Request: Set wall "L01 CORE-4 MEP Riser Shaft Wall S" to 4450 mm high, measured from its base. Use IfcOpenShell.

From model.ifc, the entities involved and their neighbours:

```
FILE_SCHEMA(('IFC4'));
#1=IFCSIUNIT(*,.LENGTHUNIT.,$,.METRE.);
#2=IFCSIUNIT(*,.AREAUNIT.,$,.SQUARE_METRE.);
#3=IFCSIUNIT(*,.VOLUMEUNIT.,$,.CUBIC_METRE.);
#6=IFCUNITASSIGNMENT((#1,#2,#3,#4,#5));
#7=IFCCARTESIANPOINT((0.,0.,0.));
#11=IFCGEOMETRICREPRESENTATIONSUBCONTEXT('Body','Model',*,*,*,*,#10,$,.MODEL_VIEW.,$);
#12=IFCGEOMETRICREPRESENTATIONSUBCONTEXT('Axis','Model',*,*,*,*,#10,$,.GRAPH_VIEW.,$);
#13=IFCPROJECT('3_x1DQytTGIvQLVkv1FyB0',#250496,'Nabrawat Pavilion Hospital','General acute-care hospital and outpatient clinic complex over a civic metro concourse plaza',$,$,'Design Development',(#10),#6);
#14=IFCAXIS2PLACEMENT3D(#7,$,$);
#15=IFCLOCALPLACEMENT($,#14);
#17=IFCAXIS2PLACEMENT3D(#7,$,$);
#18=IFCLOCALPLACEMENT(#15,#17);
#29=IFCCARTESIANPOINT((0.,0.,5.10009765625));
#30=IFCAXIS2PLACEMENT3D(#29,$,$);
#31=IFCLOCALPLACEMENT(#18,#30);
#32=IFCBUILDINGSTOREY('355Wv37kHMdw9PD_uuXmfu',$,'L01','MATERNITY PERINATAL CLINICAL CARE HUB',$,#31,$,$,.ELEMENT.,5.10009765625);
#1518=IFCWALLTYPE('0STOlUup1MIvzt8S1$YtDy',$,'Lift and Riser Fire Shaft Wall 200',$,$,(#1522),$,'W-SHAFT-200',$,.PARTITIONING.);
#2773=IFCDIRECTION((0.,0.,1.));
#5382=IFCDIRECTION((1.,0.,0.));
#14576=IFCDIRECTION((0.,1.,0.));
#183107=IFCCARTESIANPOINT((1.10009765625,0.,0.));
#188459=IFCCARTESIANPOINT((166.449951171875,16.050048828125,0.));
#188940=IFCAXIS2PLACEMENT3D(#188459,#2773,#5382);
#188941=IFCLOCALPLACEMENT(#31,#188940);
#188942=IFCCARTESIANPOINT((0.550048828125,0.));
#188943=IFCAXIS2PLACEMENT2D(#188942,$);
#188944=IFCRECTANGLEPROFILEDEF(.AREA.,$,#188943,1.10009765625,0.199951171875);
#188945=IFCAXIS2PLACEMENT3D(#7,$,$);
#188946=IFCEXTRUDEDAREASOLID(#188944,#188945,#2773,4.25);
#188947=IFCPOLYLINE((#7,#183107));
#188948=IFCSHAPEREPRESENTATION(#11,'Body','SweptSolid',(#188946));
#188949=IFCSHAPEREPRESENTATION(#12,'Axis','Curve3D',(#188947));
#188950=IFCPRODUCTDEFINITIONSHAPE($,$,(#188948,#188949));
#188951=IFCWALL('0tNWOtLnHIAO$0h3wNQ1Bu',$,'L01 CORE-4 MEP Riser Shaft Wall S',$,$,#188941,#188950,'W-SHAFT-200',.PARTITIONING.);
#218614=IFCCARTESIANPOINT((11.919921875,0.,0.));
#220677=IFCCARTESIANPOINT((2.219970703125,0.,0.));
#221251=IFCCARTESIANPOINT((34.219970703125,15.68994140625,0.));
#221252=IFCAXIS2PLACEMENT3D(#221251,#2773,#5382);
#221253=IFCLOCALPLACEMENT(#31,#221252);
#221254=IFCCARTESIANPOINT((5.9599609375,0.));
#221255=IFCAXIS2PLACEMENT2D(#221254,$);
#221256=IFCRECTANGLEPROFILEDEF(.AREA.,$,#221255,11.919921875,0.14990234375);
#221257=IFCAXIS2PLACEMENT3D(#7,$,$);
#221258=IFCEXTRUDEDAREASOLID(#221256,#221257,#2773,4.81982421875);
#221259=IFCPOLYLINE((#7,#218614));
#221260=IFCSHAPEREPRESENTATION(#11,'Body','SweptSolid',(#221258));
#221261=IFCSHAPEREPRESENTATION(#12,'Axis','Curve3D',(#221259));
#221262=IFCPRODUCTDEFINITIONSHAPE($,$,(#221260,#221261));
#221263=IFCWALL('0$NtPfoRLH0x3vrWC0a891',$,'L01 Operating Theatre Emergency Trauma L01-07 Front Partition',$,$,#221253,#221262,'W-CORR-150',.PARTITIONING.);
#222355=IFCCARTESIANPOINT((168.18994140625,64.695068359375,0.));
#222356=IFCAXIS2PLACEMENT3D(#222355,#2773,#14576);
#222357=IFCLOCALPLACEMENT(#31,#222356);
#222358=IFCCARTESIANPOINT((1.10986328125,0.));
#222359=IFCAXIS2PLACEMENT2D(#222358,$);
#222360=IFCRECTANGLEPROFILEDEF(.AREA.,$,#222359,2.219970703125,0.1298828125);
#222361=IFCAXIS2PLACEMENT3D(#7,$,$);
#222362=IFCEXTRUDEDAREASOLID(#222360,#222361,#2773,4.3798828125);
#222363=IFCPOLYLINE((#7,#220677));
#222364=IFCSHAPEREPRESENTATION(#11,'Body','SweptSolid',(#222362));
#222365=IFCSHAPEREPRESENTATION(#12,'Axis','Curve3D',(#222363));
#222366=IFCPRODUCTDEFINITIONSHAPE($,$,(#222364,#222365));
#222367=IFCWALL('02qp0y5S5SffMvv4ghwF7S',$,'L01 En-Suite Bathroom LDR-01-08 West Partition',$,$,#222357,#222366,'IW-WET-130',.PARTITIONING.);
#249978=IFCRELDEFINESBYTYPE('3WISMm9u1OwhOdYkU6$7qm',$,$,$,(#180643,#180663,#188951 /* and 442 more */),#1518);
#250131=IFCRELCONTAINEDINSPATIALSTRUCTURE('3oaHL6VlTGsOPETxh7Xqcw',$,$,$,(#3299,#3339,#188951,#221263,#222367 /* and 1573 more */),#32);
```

```python
import ifcopenshell
import ifcopenshell.geom
import ifcopenshell.util.representation
import ifcopenshell.util.shape
import ifcopenshell.util.unit

model = ifcopenshell.open("model.ifc")
unit_scale = ifcopenshell.util.unit.calculate_unit_scale(model)
settings = ifcopenshell.geom.settings()


def volume(element):
    """Net volume in cubic metres, openings subtracted."""
    shape = ifcopenshell.geom.create_shape(settings, element)
    return ifcopenshell.util.shape.get_volume(shape.geometry)


wall = model.by_guid("0tNWOtLnHIAO$0h3wNQ1Bu")
before = volume(wall)

body = ifcopenshell.util.representation.get_representation(wall, "Model", "Body")
solid = body.Items[0]
old_height = solid.Depth
solid.Depth = 4.45 / unit_scale
after = volume(wall)

print(f"height {old_height:g} -> {solid.Depth:g}, volume {before:.3f} -> {after:.3f} m3")

model.write("model_updated.ifc")
```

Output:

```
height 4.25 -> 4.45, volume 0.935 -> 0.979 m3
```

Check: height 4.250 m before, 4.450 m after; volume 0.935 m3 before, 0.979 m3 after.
